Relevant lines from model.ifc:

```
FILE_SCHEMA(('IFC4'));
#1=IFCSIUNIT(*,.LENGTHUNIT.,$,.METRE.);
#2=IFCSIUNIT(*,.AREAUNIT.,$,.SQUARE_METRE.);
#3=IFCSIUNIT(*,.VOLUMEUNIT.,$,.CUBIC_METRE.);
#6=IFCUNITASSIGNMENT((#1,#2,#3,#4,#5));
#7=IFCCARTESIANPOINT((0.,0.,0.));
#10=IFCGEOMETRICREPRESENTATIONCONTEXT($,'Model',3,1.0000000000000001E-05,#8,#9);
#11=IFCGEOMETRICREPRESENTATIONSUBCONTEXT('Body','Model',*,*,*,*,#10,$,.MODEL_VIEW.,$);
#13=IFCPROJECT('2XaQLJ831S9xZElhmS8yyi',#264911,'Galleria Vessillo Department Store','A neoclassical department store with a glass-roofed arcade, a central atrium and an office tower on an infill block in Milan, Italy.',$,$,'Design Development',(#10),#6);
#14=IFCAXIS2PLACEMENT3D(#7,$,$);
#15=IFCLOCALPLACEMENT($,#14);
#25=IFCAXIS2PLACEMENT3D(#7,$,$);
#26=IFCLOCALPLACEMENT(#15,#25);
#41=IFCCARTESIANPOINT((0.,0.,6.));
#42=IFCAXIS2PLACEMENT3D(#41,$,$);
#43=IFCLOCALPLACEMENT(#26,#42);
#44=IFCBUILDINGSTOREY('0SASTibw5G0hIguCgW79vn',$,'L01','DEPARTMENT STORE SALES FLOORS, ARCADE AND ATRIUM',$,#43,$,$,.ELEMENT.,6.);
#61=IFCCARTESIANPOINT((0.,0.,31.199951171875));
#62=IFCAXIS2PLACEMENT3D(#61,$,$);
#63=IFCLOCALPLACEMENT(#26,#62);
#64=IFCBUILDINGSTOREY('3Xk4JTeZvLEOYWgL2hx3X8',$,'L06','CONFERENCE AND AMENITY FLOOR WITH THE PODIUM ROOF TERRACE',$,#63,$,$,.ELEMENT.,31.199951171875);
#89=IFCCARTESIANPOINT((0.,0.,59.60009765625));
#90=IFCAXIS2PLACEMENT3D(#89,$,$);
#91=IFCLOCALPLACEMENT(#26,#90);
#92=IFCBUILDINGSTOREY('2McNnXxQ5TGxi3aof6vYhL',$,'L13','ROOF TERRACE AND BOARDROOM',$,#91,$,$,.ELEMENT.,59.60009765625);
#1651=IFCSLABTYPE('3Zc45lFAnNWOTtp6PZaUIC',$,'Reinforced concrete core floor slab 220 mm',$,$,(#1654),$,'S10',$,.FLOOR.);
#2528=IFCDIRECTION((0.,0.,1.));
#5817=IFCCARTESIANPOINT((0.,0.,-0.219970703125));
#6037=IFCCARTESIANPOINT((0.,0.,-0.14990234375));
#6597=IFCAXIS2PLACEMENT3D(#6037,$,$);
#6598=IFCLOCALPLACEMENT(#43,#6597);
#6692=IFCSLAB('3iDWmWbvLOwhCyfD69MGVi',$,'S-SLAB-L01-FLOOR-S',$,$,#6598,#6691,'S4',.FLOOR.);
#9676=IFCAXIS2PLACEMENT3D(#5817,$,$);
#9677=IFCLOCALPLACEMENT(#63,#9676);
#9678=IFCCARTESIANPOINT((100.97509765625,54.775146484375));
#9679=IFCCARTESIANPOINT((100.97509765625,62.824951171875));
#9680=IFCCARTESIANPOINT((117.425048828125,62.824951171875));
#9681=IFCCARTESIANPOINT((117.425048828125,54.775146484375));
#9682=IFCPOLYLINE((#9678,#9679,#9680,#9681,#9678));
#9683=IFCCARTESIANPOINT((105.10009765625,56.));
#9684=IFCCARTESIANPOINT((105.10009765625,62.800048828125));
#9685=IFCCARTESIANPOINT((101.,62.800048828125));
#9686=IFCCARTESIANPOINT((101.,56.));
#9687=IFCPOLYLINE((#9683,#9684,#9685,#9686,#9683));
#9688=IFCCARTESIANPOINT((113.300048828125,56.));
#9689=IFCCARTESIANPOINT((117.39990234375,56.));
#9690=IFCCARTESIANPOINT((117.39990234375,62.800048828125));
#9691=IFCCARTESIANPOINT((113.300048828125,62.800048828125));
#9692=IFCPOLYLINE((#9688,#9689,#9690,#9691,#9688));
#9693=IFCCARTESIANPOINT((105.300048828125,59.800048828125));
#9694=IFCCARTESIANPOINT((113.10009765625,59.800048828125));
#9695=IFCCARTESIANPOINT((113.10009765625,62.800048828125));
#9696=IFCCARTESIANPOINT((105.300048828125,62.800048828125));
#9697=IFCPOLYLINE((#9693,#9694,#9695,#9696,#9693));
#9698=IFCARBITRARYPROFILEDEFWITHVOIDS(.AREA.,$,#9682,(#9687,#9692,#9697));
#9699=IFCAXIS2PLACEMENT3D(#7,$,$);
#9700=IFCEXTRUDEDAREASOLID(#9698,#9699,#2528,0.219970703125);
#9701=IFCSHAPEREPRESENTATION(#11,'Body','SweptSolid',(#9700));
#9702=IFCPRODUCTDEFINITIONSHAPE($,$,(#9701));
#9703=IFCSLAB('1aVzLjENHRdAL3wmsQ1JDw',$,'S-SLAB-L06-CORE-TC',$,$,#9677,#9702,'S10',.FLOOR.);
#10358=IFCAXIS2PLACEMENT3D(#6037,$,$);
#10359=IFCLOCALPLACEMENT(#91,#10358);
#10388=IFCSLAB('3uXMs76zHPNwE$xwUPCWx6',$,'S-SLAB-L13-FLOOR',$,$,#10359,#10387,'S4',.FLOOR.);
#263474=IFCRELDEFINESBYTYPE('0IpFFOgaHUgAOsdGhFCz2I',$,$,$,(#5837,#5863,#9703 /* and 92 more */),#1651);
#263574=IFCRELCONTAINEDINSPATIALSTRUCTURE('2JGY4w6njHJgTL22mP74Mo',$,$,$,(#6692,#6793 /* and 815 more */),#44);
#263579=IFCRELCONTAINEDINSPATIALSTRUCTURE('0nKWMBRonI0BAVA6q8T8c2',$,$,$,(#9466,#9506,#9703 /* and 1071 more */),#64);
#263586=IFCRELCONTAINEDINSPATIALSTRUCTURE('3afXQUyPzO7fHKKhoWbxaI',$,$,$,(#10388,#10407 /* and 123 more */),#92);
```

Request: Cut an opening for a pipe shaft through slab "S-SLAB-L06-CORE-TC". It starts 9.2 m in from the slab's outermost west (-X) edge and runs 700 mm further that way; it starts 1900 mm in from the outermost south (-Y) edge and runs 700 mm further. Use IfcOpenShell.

```python
import numpy as np
import ifcopenshell
import ifcopenshell.api.feature
import ifcopenshell.api.geometry
import ifcopenshell.api.root
import ifcopenshell.geom
import ifcopenshell.util.placement
import ifcopenshell.util.representation
import ifcopenshell.util.shape
import ifcopenshell.util.unit

model = ifcopenshell.open("model.ifc")
unit_scale = ifcopenshell.util.unit.calculate_unit_scale(model)
settings = ifcopenshell.geom.settings()


def volume(element):
    """Net volume in cubic metres, openings subtracted."""
    shape = ifcopenshell.geom.create_shape(settings, element)
    return ifcopenshell.util.shape.get_volume(shape.geometry)


slab = model.by_guid("1aVzLjENHRdAL3wmsQ1JDw")
before = volume(slab)

# Extent in the slab's own axes, in metres. The edges named are its -X and -Y sides.
slab_shape = ifcopenshell.geom.create_shape(settings, slab)
vertices = ifcopenshell.util.shape.get_vertices(slab_shape.geometry)
x_min, y_min, bottom = vertices.min(axis=0)
top = vertices[:, 2].max()

opening = ifcopenshell.api.root.create_entity(model, ifc_class="IfcOpeningElement", name="Pipe shaft opening", predefined_type="OPENING")
context = ifcopenshell.util.representation.get_context(model, "Model", "Body", "MODEL_VIEW")
width, depth = 0.7, 0.7
outline = [(0.0, 0.0), (width, 0.0), (width, depth), (0.0, depth), (0.0, 0.0)]
# Overshoot both faces by 50 mm so the cut is clean.
shape = ifcopenshell.api.geometry.add_slab_representation(
    model, context=context, depth=top - bottom + 0.1, polyline=outline
)
ifcopenshell.api.geometry.assign_representation(model, product=opening, representation=shape)

matrix = ifcopenshell.util.placement.get_local_placement(slab.ObjectPlacement)
matrix[:, 3] = matrix @ np.append(np.array([x_min + 9.2, y_min + 1.9, bottom - 0.05]) / unit_scale, 1.0)
ifcopenshell.api.geometry.edit_object_placement(model, product=opening, matrix=matrix, is_si=False)
ifcopenshell.api.feature.add_feature(model, feature=opening, element=slab)

after = volume(slab)

print(f"slab volume {before:.3f} -> {after:.3f} m3")

model.write("model_updated.ifc")
```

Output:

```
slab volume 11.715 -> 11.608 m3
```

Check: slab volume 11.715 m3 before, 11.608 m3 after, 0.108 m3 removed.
